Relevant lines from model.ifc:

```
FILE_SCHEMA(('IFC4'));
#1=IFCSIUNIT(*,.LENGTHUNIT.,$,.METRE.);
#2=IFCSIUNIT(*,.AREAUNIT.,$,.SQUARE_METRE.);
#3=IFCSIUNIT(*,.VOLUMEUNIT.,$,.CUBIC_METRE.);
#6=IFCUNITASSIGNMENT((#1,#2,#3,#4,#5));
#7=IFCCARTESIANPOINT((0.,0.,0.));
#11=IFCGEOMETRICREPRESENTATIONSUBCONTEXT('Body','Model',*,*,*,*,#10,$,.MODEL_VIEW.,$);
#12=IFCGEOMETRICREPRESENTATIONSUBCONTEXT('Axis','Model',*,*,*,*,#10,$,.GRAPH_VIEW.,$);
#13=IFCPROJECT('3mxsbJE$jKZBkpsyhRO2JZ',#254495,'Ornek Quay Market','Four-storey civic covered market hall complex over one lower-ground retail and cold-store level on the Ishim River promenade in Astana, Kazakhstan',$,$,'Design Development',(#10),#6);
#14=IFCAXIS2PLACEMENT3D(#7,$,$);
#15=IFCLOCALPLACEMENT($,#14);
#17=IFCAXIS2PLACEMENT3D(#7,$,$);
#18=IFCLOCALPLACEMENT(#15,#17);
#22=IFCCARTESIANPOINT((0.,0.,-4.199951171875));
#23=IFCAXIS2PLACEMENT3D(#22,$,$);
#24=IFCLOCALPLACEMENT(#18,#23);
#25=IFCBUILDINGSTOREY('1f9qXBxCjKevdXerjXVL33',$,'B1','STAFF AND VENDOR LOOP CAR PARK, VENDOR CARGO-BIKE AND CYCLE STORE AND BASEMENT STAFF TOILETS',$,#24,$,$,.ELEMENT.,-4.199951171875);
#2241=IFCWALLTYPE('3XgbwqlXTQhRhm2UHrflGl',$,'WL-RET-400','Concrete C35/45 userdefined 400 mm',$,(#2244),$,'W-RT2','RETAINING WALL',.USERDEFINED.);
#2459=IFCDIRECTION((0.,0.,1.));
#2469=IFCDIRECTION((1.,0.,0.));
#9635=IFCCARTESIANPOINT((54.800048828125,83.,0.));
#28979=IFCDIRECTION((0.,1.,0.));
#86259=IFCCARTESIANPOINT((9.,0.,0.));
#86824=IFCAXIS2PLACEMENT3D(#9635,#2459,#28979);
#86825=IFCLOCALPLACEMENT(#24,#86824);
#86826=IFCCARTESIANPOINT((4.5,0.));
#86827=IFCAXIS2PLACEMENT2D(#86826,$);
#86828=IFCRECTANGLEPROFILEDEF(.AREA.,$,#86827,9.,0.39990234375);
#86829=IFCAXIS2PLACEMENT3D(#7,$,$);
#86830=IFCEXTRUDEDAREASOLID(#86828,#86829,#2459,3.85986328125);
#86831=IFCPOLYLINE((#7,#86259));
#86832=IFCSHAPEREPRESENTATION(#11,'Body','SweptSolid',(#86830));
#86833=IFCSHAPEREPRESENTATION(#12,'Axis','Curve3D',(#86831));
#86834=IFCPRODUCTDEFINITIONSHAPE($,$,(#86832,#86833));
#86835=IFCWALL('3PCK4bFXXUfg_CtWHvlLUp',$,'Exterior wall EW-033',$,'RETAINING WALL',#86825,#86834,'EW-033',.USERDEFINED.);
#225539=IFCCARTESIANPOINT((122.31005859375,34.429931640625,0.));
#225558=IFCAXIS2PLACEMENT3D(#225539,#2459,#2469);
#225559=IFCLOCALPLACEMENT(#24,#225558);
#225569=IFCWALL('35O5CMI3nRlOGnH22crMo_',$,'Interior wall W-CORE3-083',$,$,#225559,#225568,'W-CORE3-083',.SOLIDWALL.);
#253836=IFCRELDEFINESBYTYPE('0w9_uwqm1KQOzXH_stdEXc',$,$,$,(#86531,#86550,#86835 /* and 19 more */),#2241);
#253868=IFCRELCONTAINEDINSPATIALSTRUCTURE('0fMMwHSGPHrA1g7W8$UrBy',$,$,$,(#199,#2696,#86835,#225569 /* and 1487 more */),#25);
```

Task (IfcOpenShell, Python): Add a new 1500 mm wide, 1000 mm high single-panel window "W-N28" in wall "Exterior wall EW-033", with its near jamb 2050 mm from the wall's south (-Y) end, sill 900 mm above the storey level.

```python
import numpy as np
import ifcopenshell
import ifcopenshell.api.feature
import ifcopenshell.api.geometry
import ifcopenshell.api.root
import ifcopenshell.api.spatial
import ifcopenshell.geom
import ifcopenshell.util.element
import ifcopenshell.util.placement
import ifcopenshell.util.representation
import ifcopenshell.util.shape
import ifcopenshell.util.unit

model = ifcopenshell.open("model.ifc")
unit_scale = ifcopenshell.util.unit.calculate_unit_scale(model)
settings = ifcopenshell.geom.settings()


def volume(element):
    """Net volume in cubic metres, openings subtracted."""
    shape = ifcopenshell.geom.create_shape(settings, element)
    return ifcopenshell.util.shape.get_volume(shape.geometry)


wall = model.by_guid("3PCK4bFXXUfg_CtWHvlLUp")
storey = ifcopenshell.util.element.get_container(wall, ifc_class="IfcBuildingStorey")
context = ifcopenshell.util.representation.get_context(model, "Model", "Body", "MODEL_VIEW")
before = volume(wall)

width, height, from_end, sill = 1.5, 1, 2.05, 0.9  # metres

# The wall runs along its own X axis, and the end named is its -X end.
wall_shape = ifcopenshell.geom.create_shape(settings, wall)
x, y, z = ifcopenshell.util.shape.get_vertices(wall_shape.geometry).T
start = x.min() + from_end
face, thickness = float(y.min()), float(y.max() - y.min())
wall_matrix = ifcopenshell.util.placement.get_local_placement(wall.ObjectPlacement)
level = ifcopenshell.util.placement.get_local_placement(storey.ObjectPlacement)[2, 3]


def in_wall(x, y):
    """Placement at x, y metres in the wall's axes, at sill height."""
    matrix = wall_matrix.copy()
    matrix[:, 3] = wall_matrix @ np.array([x / unit_scale, y / unit_scale, 0.0, 1.0])
    matrix[2, 3] = level + sill / unit_scale
    return matrix


# Opening: a box that overshoots both wall faces by 50 mm.
opening = ifcopenshell.api.root.create_entity(model, ifc_class="IfcOpeningElement", predefined_type="OPENING")
box = ifcopenshell.api.geometry.add_wall_representation(
    model, context=context, length=width, height=height, thickness=thickness + 0.1
)
ifcopenshell.api.geometry.assign_representation(model, product=opening, representation=box)
ifcopenshell.api.geometry.edit_object_placement(model, product=opening, matrix=in_wall(start, face - 0.05), is_si=False)
ifcopenshell.api.feature.add_feature(model, feature=opening, element=wall)

window = ifcopenshell.api.root.create_entity(model, ifc_class="IfcWindow", name="W-N28", predefined_type="WINDOW")
window.OverallWidth, window.OverallHeight = width / unit_scale, height / unit_scale
window.PartitioningType = "SINGLE_PANEL"
body = ifcopenshell.api.geometry.add_window_representation(
    model,
    context=context,
    overall_width=window.OverallWidth,
    overall_height=window.OverallHeight,
    partition_type="SINGLE_PANEL",
)
ifcopenshell.api.geometry.assign_representation(model, product=window, representation=body)
ifcopenshell.api.spatial.assign_container(model, products=[window], relating_structure=storey)
ifcopenshell.api.feature.add_filling(model, opening=opening, element=window)

# Centre the window in the wall's thickness.
ifcopenshell.api.geometry.edit_object_placement(model, product=window, matrix=in_wall(start, face), is_si=False)
window_shape = ifcopenshell.geom.create_shape(settings, window)
depth = ifcopenshell.util.shape.get_vertices(window_shape.geometry)[:, 1]
offset = face + thickness / 2 - (depth.min() + depth.max()) / 2
ifcopenshell.api.geometry.edit_object_placement(model, product=window, matrix=in_wall(start, offset), is_si=False)

after = volume(wall)

print(f"wall volume {before:.3f} -> {after:.3f} m3")

model.write("model_updated.ifc")
```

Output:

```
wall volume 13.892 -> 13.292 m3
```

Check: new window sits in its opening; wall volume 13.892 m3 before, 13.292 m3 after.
